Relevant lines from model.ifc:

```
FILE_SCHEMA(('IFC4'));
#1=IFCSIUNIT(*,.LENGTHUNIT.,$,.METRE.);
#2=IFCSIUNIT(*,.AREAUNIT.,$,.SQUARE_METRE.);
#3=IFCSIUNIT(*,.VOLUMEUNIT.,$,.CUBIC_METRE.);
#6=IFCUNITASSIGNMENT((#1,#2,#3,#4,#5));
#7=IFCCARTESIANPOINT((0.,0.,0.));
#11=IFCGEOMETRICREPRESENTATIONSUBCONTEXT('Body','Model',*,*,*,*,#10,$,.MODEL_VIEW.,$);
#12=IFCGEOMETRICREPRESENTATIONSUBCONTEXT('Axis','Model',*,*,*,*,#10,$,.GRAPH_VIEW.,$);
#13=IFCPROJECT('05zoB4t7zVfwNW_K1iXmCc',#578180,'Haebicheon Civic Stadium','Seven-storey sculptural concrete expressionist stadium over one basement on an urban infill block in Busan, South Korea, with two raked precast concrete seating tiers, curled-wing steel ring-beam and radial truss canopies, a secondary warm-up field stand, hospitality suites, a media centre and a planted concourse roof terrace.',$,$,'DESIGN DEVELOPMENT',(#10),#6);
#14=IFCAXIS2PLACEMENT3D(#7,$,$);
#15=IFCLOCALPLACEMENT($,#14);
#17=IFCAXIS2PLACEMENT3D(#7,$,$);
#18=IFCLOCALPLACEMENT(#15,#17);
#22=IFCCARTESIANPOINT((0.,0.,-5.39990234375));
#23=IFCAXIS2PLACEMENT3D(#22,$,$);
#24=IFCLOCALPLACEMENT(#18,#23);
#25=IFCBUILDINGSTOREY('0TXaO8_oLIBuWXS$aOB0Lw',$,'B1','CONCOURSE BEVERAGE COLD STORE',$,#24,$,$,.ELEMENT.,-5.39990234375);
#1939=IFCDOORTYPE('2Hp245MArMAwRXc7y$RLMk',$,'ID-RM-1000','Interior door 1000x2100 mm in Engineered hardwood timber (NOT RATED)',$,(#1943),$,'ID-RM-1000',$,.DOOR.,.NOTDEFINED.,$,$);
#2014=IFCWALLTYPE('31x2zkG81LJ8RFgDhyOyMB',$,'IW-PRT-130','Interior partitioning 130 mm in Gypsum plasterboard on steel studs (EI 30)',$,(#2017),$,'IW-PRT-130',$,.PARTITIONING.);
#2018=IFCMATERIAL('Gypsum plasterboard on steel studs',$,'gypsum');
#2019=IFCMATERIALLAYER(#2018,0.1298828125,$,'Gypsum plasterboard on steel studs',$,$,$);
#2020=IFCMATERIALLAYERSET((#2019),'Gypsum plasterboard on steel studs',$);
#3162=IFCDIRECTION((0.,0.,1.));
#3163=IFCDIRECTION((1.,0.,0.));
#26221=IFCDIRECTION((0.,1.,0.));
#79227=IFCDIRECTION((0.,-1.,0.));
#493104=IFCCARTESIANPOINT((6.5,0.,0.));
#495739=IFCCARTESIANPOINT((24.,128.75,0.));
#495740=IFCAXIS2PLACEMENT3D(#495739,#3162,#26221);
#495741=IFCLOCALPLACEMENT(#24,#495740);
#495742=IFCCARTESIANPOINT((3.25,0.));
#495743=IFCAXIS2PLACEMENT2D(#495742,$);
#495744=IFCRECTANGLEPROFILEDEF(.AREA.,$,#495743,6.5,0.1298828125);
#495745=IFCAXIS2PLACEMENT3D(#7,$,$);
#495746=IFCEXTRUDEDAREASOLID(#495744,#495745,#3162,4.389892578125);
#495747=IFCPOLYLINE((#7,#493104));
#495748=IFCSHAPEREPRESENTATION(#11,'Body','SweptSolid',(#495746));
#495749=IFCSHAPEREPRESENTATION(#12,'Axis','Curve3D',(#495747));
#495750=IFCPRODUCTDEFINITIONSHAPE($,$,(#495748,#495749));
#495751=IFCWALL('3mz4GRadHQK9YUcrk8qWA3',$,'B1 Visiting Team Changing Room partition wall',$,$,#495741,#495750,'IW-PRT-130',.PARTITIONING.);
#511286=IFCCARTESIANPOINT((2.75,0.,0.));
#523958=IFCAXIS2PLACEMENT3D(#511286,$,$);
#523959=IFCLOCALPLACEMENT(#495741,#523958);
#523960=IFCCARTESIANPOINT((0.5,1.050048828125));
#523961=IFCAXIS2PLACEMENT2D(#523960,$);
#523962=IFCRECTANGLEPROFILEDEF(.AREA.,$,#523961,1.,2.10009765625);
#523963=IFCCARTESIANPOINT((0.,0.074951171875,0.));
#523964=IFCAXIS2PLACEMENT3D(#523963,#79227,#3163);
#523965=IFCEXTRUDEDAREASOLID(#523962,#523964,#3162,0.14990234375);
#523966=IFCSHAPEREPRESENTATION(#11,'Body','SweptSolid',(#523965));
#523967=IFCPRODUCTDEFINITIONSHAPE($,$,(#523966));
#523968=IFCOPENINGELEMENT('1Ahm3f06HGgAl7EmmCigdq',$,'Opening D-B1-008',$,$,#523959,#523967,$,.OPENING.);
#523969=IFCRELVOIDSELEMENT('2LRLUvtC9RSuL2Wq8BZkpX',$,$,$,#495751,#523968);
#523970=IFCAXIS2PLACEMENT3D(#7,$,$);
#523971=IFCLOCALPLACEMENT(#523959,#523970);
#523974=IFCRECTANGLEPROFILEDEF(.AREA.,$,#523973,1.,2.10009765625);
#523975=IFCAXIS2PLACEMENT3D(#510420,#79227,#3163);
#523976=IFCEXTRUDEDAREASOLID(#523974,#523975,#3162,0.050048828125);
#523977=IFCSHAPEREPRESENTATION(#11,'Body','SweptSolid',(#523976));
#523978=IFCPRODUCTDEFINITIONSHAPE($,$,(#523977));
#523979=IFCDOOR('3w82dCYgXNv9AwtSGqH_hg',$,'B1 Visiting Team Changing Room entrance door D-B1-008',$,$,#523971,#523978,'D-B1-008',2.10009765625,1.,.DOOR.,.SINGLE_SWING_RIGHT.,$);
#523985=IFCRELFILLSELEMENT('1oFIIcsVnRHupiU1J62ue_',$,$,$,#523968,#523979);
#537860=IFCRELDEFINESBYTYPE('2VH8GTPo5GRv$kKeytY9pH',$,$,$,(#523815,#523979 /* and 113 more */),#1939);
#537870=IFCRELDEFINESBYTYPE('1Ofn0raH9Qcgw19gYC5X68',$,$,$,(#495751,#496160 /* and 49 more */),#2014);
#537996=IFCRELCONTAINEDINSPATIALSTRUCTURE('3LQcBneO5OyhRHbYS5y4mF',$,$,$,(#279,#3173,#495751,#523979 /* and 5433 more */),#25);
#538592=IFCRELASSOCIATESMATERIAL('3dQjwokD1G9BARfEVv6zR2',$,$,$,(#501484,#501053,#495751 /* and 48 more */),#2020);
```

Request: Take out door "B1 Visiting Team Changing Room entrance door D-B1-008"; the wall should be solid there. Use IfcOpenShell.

```python
import ifcopenshell
import ifcopenshell.api.feature
import ifcopenshell.api.root
import ifcopenshell.geom
import ifcopenshell.util.shape

model = ifcopenshell.open("model.ifc")
settings = ifcopenshell.geom.settings()


def volume(element):
    """Net volume in cubic metres, openings subtracted."""
    shape = ifcopenshell.geom.create_shape(settings, element)
    return ifcopenshell.util.shape.get_volume(shape.geometry)


door = model.by_guid("3w82dCYgXNv9AwtSGqH_hg")
opening = door.FillsVoids[0].RelatingOpeningElement
wall = opening.VoidsElements[0].RelatingBuildingElement
before = volume(wall)

ifcopenshell.api.root.remove_product(model, product=door)
ifcopenshell.api.feature.remove_feature(model, feature=opening)

after = volume(wall)

print(f"wall volume {before:.3f} -> {after:.3f} m3")

model.write("model_updated.ifc")
```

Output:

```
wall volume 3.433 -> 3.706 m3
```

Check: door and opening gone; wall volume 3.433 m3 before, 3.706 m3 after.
